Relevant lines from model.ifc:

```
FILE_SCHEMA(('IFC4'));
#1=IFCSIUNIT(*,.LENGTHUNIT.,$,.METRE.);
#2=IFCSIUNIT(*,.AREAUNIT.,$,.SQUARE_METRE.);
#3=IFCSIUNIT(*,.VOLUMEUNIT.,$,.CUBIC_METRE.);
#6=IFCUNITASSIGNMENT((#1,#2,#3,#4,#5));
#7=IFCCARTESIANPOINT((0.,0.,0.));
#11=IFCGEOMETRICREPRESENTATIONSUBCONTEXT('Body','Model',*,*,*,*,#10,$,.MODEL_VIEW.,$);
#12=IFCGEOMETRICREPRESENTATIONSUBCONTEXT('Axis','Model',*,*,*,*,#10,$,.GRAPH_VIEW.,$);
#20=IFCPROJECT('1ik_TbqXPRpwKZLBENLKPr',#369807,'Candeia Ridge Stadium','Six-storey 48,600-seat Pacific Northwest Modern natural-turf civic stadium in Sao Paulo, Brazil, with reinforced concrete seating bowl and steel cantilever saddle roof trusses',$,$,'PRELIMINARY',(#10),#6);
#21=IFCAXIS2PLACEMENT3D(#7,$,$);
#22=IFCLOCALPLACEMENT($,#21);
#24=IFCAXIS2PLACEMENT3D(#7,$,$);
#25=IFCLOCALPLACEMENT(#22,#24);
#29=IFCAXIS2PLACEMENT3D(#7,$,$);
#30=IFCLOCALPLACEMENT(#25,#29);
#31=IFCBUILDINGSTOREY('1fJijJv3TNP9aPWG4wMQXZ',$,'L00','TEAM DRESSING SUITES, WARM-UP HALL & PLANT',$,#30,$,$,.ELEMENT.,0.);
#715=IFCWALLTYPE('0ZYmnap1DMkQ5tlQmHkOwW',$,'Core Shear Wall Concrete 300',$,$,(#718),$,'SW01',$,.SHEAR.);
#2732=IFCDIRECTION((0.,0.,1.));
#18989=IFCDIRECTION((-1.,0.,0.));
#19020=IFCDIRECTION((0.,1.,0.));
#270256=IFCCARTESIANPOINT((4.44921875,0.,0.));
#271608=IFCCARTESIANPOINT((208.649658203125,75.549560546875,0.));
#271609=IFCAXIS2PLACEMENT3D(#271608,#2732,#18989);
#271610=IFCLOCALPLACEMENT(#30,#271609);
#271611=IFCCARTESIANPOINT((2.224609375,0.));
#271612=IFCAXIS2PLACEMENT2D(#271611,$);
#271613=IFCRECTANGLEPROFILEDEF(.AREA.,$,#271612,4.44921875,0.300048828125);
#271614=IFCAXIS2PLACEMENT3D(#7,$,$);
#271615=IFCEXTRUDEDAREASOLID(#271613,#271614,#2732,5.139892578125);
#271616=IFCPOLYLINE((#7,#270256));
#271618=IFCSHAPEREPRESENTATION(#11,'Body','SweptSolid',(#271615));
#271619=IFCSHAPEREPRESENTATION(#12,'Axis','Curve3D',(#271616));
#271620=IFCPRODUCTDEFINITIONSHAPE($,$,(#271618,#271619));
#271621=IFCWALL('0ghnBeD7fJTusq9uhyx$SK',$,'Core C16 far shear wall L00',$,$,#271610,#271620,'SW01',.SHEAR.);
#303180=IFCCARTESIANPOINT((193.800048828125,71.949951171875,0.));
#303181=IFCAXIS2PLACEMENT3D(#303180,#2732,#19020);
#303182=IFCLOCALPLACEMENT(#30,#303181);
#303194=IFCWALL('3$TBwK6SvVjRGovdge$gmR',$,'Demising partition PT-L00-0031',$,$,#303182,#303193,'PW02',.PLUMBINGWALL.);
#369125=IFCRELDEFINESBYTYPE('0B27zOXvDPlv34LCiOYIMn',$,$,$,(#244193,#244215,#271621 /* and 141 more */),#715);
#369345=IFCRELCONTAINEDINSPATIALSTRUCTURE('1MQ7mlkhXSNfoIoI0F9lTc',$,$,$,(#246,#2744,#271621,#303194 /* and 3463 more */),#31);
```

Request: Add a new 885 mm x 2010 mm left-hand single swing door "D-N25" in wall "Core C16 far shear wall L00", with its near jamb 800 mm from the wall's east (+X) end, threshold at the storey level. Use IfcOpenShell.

```python
import numpy as np
import ifcopenshell
import ifcopenshell.api.feature
import ifcopenshell.api.geometry
import ifcopenshell.api.root
import ifcopenshell.api.spatial
import ifcopenshell.geom
import ifcopenshell.util.element
import ifcopenshell.util.placement
import ifcopenshell.util.representation
import ifcopenshell.util.shape
import ifcopenshell.util.unit

model = ifcopenshell.open("model.ifc")
unit_scale = ifcopenshell.util.unit.calculate_unit_scale(model)
settings = ifcopenshell.geom.settings()


def volume(element):
    """Net volume in cubic metres, openings subtracted."""
    shape = ifcopenshell.geom.create_shape(settings, element)
    return ifcopenshell.util.shape.get_volume(shape.geometry)


wall = model.by_guid("0ghnBeD7fJTusq9uhyx$SK")
storey = ifcopenshell.util.element.get_container(wall, ifc_class="IfcBuildingStorey")
context = ifcopenshell.util.representation.get_context(model, "Model", "Body", "MODEL_VIEW")
before = volume(wall)

width, height, from_end, sill = 0.885, 2.01, 0.8, 0.0  # metres

# The wall runs along its own X axis, and the end named is its -X end.
wall_shape = ifcopenshell.geom.create_shape(settings, wall)
x, y, z = ifcopenshell.util.shape.get_vertices(wall_shape.geometry).T
start = x.min() + from_end
face, thickness = float(y.min()), float(y.max() - y.min())
wall_matrix = ifcopenshell.util.placement.get_local_placement(wall.ObjectPlacement)
level = ifcopenshell.util.placement.get_local_placement(storey.ObjectPlacement)[2, 3]


def in_wall(x, y):
    """Placement at x, y metres in the wall's axes, at sill height."""
    matrix = wall_matrix.copy()
    matrix[:, 3] = wall_matrix @ np.array([x / unit_scale, y / unit_scale, 0.0, 1.0])
    matrix[2, 3] = level + sill / unit_scale
    return matrix


# Opening: a box that overshoots both wall faces by 50 mm.
opening = ifcopenshell.api.root.create_entity(model, ifc_class="IfcOpeningElement", predefined_type="OPENING")
box = ifcopenshell.api.geometry.add_wall_representation(
    model, context=context, length=width, height=height, thickness=thickness + 0.1
)
ifcopenshell.api.geometry.assign_representation(model, product=opening, representation=box)
ifcopenshell.api.geometry.edit_object_placement(model, product=opening, matrix=in_wall(start, face - 0.05), is_si=False)
ifcopenshell.api.feature.add_feature(model, feature=opening, element=wall)

door = ifcopenshell.api.root.create_entity(model, ifc_class="IfcDoor", name="D-N25", predefined_type="DOOR")
door.OverallWidth, door.OverallHeight = width / unit_scale, height / unit_scale
door.OperationType = "SINGLE_SWING_LEFT"
body = ifcopenshell.api.geometry.add_door_representation(
    model,
    context=context,
    overall_width=door.OverallWidth,
    overall_height=door.OverallHeight,
    operation_type="SINGLE_SWING_LEFT",
    lining_properties={"LiningDepth": thickness / unit_scale, "ThresholdDepth": thickness / unit_scale},
)
ifcopenshell.api.geometry.assign_representation(model, product=door, representation=body)
ifcopenshell.api.spatial.assign_container(model, products=[door], relating_structure=storey)
ifcopenshell.api.feature.add_filling(model, opening=opening, element=door)

# The lining spans the wall, so the door starts at the wall face.
ifcopenshell.api.geometry.edit_object_placement(model, product=door, matrix=in_wall(start, face), is_si=False)

after = volume(wall)

print(f"wall volume {before:.3f} -> {after:.3f} m3")

model.write("model_v2.ifc")
```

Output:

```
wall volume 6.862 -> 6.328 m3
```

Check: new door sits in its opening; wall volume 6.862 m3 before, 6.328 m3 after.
